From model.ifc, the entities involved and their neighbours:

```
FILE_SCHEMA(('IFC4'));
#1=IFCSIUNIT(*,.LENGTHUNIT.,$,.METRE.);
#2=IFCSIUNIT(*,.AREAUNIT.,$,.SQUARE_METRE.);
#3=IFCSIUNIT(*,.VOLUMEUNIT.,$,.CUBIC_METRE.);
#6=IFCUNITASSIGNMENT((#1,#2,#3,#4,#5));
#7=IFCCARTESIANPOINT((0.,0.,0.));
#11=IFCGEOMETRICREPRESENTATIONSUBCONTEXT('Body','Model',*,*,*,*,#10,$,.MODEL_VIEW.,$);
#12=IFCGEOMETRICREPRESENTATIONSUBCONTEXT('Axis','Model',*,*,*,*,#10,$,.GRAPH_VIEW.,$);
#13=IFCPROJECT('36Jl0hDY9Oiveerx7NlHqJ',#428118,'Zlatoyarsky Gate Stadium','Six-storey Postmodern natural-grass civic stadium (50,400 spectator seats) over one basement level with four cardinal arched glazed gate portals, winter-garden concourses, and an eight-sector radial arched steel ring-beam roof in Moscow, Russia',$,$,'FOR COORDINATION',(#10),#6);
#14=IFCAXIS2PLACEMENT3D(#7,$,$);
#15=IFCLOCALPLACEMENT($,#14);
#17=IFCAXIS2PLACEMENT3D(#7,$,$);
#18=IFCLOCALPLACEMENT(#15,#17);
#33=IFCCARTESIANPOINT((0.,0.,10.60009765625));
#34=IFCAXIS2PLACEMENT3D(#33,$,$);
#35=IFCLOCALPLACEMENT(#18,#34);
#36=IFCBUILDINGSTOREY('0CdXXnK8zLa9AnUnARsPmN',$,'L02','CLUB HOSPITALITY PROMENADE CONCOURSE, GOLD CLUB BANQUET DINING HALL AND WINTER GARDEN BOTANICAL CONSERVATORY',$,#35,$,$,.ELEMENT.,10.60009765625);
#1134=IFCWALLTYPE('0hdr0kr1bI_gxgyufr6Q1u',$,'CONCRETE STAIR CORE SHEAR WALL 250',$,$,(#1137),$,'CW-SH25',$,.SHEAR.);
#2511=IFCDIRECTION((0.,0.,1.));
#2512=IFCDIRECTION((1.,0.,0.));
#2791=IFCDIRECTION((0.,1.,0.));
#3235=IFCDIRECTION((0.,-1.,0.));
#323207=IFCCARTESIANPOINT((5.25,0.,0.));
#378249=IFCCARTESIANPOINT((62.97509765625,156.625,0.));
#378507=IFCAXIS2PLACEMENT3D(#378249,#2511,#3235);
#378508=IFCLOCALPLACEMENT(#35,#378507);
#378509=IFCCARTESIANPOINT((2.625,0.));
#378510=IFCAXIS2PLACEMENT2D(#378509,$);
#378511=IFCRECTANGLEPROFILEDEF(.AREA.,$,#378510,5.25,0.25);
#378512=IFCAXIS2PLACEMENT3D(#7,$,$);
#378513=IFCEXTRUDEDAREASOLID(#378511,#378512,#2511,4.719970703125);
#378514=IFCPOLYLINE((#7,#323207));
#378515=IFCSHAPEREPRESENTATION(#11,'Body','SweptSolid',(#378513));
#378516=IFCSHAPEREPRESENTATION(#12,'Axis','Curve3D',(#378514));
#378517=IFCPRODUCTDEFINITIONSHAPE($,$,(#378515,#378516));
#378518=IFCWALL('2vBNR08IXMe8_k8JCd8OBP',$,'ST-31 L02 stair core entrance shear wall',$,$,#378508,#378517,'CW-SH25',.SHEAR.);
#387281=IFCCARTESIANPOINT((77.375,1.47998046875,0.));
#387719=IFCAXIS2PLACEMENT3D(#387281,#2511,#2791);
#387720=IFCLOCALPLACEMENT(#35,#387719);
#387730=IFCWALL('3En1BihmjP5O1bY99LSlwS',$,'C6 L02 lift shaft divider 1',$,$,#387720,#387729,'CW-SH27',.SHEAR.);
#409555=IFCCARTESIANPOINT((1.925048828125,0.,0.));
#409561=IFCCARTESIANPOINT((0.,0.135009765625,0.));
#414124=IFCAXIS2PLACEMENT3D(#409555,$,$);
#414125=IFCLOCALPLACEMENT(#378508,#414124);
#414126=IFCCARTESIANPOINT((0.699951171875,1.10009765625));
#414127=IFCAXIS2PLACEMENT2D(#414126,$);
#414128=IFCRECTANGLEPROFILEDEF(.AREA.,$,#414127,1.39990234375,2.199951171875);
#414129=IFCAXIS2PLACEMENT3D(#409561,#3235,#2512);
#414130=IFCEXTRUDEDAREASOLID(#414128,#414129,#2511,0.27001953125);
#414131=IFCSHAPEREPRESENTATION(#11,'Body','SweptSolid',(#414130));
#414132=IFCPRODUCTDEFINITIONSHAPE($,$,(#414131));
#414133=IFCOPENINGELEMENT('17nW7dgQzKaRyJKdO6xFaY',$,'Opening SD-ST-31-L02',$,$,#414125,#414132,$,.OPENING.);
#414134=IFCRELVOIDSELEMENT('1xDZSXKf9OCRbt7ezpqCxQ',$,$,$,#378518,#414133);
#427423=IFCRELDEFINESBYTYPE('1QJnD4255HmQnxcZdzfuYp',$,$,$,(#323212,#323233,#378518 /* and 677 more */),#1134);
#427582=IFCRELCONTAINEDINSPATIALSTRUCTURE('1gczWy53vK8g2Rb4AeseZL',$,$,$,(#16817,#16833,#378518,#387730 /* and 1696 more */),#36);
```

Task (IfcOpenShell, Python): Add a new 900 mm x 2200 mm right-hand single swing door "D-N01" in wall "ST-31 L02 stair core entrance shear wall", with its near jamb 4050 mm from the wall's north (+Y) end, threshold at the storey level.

```python
import numpy as np
import ifcopenshell
import ifcopenshell.api.feature
import ifcopenshell.api.geometry
import ifcopenshell.api.root
import ifcopenshell.api.spatial
import ifcopenshell.geom
import ifcopenshell.util.element
import ifcopenshell.util.placement
import ifcopenshell.util.representation
import ifcopenshell.util.shape
import ifcopenshell.util.unit

model = ifcopenshell.open("model.ifc")
unit_scale = ifcopenshell.util.unit.calculate_unit_scale(model)
settings = ifcopenshell.geom.settings()


def volume(element):
    """Net volume in cubic metres, openings subtracted."""
    shape = ifcopenshell.geom.create_shape(settings, element)
    return ifcopenshell.util.shape.get_volume(shape.geometry)


wall = model.by_guid("2vBNR08IXMe8_k8JCd8OBP")
storey = ifcopenshell.util.element.get_container(wall, ifc_class="IfcBuildingStorey")
context = ifcopenshell.util.representation.get_context(model, "Model", "Body", "MODEL_VIEW")
before = volume(wall)

width, height, from_end, sill = 0.9, 2.2, 4.05, 0.0  # metres

# The wall runs along its own X axis, and the end named is its -X end.
wall_shape = ifcopenshell.geom.create_shape(settings, wall)
x, y, z = ifcopenshell.util.shape.get_vertices(wall_shape.geometry).T
start = x.min() + from_end
face, thickness = float(y.min()), float(y.max() - y.min())
wall_matrix = ifcopenshell.util.placement.get_local_placement(wall.ObjectPlacement)
level = ifcopenshell.util.placement.get_local_placement(storey.ObjectPlacement)[2, 3]


def in_wall(x, y):
    """Placement at x, y metres in the wall's axes, at sill height."""
    matrix = wall_matrix.copy()
    matrix[:, 3] = wall_matrix @ np.array([x / unit_scale, y / unit_scale, 0.0, 1.0])
    matrix[2, 3] = level + sill / unit_scale
    return matrix


# Opening: a box that overshoots both wall faces by 50 mm.
opening = ifcopenshell.api.root.create_entity(model, ifc_class="IfcOpeningElement", predefined_type="OPENING")
box = ifcopenshell.api.geometry.add_wall_representation(
    model, context=context, length=width, height=height, thickness=thickness + 0.1
)
ifcopenshell.api.geometry.assign_representation(model, product=opening, representation=box)
ifcopenshell.api.geometry.edit_object_placement(model, product=opening, matrix=in_wall(start, face - 0.05), is_si=False)
ifcopenshell.api.feature.add_feature(model, feature=opening, element=wall)

door = ifcopenshell.api.root.create_entity(model, ifc_class="IfcDoor", name="D-N01", predefined_type="DOOR")
door.OverallWidth, door.OverallHeight = width / unit_scale, height / unit_scale
door.OperationType = "SINGLE_SWING_RIGHT"
body = ifcopenshell.api.geometry.add_door_representation(
    model,
    context=context,
    overall_width=door.OverallWidth,
    overall_height=door.OverallHeight,
    operation_type="SINGLE_SWING_RIGHT",
    lining_properties={"LiningDepth": thickness / unit_scale, "ThresholdDepth": thickness / unit_scale},
)
ifcopenshell.api.geometry.assign_representation(model, product=door, representation=body)
ifcopenshell.api.spatial.assign_container(model, products=[door], relating_structure=storey)
ifcopenshell.api.feature.add_filling(model, opening=opening, element=door)

# The lining spans the wall, so the door starts at the wall face.
ifcopenshell.api.geometry.edit_object_placement(model, product=door, matrix=in_wall(start, face), is_si=False)

after = volume(wall)

print(f"wall volume {before:.3f} -> {after:.3f} m3")

model.write("model_edited.ifc")
```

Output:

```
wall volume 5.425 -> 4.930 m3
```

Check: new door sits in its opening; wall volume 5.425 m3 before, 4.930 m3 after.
